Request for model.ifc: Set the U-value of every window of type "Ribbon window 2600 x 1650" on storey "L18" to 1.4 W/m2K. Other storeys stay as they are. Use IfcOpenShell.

First a look at what the model holds.

```python
import ifcopenshell
import ifcopenshell.util.element

model = ifcopenshell.open("model.ifc")
print(model.schema)
storey = next(s for s in model.by_type("IfcBuildingStorey") if s.Name == "L18")
windows = [e for e in ifcopenshell.util.element.get_decomposition(storey) if e.is_a("IfcWindow")]
seen = {}
for e in windows:
    element_type = ifcopenshell.util.element.get_type(e)
    key = (element_type.Name if element_type != e and element_type else None, ifcopenshell.util.element.get_pset(e, "Pset_WindowCommon", "ThermalTransmittance"))
    seen[key] = seen.get(key, 0) + 1
for (name, value), count in sorted(seen.items(), key=str):
    print(count, "x", name, "|", value)
```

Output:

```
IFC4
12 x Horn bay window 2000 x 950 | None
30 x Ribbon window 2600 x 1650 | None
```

```python
import ifcopenshell
import ifcopenshell.api.pset
import ifcopenshell.util.element

model = ifcopenshell.open("model.ifc")

storey = next(s for s in model.by_type("IfcBuildingStorey") if s.Name == "L18")
windows = [e for e in ifcopenshell.util.element.get_decomposition(storey) if e.is_a("IfcWindow")]

count = 0
for e in windows:
    element_type = ifcopenshell.util.element.get_type(e)
    if element_type in (None, e) or element_type.Name != "Ribbon window 2600 x 1650":
        continue
    found = ifcopenshell.util.element.get_pset(e, "Pset_WindowCommon", should_inherit=False)
    if found:
        pset = model.by_id(found["id"])
        if len(ifcopenshell.util.element.get_elements_by_pset(pset)) > 1:
            pset = ifcopenshell.api.pset.unshare_pset(model, products=[e], pset=pset)[0]
    else:
        pset = ifcopenshell.api.pset.add_pset(model, product=e, name="Pset_WindowCommon")
    ifcopenshell.api.pset.edit_pset(model, pset=pset, properties={"ThermalTransmittance": 1.4})
    count += 1

print(count, "windows updated")

model.write("model_edited.ifc")
```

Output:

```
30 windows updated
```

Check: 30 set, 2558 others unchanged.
